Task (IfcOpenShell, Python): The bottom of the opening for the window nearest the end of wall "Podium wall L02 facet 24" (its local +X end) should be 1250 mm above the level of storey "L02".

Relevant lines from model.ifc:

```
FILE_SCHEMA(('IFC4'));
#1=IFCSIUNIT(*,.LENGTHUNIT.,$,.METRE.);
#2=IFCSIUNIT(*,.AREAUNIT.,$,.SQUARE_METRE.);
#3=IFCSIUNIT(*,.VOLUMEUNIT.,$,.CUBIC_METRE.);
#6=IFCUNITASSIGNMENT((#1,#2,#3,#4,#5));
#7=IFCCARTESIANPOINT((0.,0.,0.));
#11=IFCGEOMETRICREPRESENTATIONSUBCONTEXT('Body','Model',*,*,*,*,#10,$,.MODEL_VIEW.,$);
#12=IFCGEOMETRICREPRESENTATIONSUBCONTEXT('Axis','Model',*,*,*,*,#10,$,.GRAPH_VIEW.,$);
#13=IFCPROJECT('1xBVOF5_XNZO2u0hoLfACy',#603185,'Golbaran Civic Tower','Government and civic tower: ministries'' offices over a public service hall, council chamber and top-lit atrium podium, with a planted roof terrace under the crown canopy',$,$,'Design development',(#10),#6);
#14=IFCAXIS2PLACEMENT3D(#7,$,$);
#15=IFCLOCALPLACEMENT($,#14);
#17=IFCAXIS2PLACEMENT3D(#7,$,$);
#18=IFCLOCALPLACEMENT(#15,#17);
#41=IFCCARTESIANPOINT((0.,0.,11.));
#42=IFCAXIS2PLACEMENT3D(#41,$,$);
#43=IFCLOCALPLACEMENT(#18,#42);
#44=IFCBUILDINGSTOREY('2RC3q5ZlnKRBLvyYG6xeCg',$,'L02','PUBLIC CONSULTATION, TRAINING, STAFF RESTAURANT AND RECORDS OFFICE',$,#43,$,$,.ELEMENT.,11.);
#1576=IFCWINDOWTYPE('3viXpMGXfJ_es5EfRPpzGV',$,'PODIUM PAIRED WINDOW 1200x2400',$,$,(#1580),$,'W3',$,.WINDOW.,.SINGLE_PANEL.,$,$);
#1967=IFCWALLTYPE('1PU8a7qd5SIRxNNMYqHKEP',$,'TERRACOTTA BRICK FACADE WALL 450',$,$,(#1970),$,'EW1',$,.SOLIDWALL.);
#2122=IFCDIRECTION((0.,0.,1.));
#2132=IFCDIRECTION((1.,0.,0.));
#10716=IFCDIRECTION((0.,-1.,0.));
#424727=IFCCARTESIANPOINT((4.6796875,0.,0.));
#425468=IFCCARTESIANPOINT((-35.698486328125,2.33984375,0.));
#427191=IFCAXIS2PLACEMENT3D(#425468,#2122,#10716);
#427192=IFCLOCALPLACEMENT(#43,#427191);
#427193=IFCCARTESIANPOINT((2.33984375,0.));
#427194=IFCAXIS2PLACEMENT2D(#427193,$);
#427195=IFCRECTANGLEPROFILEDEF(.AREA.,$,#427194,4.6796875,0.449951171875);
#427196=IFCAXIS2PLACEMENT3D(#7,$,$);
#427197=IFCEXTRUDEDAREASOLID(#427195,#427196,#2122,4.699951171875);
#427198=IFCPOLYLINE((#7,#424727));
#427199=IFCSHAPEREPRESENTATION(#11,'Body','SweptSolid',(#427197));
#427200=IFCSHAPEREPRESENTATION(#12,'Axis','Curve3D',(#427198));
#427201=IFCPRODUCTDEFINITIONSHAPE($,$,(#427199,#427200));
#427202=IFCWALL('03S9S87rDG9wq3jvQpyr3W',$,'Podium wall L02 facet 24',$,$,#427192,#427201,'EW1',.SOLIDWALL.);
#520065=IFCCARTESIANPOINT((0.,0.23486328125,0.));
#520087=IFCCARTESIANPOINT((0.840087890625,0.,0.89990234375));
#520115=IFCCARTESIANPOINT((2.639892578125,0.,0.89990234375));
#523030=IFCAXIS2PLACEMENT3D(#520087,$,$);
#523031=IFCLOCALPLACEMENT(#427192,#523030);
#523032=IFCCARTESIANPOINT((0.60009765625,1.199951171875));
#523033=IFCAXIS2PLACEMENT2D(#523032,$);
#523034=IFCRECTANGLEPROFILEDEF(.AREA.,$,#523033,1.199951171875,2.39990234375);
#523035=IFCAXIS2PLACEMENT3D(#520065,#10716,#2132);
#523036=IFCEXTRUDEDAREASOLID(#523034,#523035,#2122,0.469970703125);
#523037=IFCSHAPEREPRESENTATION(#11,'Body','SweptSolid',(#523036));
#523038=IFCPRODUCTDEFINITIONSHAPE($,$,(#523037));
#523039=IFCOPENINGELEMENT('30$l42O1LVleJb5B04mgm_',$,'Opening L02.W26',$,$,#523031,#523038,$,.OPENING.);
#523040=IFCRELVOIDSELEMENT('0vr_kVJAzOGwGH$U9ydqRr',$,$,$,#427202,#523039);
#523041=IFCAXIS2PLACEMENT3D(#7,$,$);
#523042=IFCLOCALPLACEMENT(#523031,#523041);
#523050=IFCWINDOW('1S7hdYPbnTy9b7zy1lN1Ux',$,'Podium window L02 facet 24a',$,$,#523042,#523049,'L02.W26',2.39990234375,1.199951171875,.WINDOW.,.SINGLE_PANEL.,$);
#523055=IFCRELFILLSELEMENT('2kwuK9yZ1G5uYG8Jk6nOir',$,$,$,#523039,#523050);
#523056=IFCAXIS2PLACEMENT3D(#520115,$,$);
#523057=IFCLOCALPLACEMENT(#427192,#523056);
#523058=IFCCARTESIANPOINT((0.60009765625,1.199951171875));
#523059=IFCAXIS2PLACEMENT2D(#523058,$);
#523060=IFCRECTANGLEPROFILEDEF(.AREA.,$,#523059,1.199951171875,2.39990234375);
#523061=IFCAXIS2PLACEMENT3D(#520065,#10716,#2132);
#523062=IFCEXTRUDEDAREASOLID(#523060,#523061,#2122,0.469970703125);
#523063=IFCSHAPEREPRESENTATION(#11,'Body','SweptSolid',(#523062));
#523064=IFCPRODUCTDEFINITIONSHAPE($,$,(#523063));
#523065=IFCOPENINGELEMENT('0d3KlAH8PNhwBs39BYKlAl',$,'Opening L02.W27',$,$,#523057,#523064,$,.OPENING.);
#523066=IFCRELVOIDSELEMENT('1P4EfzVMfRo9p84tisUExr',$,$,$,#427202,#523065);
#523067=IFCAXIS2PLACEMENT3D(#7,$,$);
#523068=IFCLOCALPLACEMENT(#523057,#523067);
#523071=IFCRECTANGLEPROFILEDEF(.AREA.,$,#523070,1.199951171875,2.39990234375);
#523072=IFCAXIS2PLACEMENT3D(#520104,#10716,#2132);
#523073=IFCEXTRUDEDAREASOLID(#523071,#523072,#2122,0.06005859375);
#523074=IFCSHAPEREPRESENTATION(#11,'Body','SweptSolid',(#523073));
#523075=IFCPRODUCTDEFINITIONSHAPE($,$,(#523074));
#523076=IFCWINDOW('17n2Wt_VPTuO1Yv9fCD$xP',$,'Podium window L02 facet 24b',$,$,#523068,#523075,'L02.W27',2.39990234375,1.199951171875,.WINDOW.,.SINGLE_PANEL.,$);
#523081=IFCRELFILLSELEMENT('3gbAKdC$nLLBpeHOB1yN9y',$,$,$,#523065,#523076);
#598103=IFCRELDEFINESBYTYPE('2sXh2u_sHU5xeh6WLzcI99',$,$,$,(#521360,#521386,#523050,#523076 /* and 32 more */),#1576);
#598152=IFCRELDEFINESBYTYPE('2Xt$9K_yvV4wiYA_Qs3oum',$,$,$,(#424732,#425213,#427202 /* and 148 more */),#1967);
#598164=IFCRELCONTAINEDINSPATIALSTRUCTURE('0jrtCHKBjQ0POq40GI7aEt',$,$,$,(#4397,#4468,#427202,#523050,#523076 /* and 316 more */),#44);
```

```python
import numpy as np
import ifcopenshell
import ifcopenshell.api.geometry
import ifcopenshell.geom
import ifcopenshell.util.element
import ifcopenshell.util.placement
import ifcopenshell.util.shape
import ifcopenshell.util.unit

model = ifcopenshell.open("model.ifc")
unit_scale = ifcopenshell.util.unit.calculate_unit_scale(model)

window = model.by_guid("17n2Wt_VPTuO1Yv9fCD$xP")
opening = window.FillsVoids[0].RelatingOpeningElement
storey = ifcopenshell.util.element.get_container(window, ifc_class="IfcBuildingStorey")
level = ifcopenshell.util.placement.get_local_placement(storey.ObjectPlacement)[2, 3]

# The opening's origin need not be at the sill, so measure its lowest point.
shape = ifcopenshell.geom.create_shape(ifcopenshell.geom.settings(), opening)
bottom = ifcopenshell.util.shape.get_shape_bottom_elevation(shape, shape.geometry) / unit_scale
dz = level + 1.25 / unit_scale - bottom

shift = np.array([0.0, 0.0, dz])
# The window is placed relative to its opening, so it follows when the opening moves.
matrix = ifcopenshell.util.placement.get_local_placement(opening.ObjectPlacement)
matrix[:3, 3] += shift
ifcopenshell.api.geometry.edit_object_placement(
    model, product=opening, matrix=matrix, is_si=False, should_transform_children=True
)

print(f"moved by {dz * unit_scale:+.3f} m")

model.write("model_edited.ifc")
```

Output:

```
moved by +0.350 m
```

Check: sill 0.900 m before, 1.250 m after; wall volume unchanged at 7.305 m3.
